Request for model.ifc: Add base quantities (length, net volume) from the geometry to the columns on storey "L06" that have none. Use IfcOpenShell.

First a look at what the model holds.

```python
import ifcopenshell
import ifcopenshell.util.element
import ifcopenshell.util.unit

model = ifcopenshell.open("model.ifc")
print(model.schema)
for unit_type in ("LENGTHUNIT", "AREAUNIT", "VOLUMEUNIT"):
    print(unit_type, ifcopenshell.util.unit.calculate_unit_scale(model, unit_type))
storey = next(s for s in model.by_type("IfcBuildingStorey") if s.Name == "L06")
columns = [e for e in ifcopenshell.util.element.get_decomposition(storey) if e.is_a("IfcColumn")]
for e in sorted(columns, key=lambda e: e.id()):
    print(e.id(), e.is_a(), e.Name, list(ifcopenshell.util.element.get_psets(e, qtos_only=True)), sep=" | ")
```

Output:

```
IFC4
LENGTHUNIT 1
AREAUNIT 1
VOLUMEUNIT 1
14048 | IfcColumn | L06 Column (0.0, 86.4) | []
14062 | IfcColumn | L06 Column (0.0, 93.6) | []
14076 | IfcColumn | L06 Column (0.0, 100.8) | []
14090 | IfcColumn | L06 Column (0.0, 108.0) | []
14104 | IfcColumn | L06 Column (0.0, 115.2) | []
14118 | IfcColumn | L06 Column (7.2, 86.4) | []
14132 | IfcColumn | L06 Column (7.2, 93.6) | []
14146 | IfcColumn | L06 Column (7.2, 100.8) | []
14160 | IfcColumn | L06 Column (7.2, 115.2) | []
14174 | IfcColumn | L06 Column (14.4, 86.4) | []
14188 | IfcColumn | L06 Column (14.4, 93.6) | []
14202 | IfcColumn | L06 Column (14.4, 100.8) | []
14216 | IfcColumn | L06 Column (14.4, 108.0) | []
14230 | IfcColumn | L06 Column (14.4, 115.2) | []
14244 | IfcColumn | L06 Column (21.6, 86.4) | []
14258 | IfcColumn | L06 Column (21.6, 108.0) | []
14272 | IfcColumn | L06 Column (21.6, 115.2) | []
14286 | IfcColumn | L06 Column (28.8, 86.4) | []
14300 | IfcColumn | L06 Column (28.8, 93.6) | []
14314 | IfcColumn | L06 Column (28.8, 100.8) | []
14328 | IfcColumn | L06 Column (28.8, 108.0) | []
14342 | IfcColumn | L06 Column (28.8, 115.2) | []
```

```python
import ifcopenshell
import ifcopenshell.api.pset
import ifcopenshell.geom
import ifcopenshell.util.element
import ifcopenshell.util.shape
import ifcopenshell.util.unit

model = ifcopenshell.open("model.ifc")
unit_scale = ifcopenshell.util.unit.calculate_unit_scale(model)
volume_scale = ifcopenshell.util.unit.calculate_unit_scale(model, "VOLUMEUNIT")
settings = ifcopenshell.geom.settings()

storey = next(s for s in model.by_type("IfcBuildingStorey") if s.Name == "L06")
columns = [e for e in ifcopenshell.util.element.get_decomposition(storey) if e.is_a("IfcColumn")]

for e in sorted(columns, key=lambda e: e.id()):
    if ifcopenshell.util.element.get_psets(e, qtos_only=True, should_inherit=False):
        continue
    # Geometry comes back in metres, in the element's own axes.
    shape = ifcopenshell.geom.create_shape(settings, e)
    values = {
        "Length": ifcopenshell.util.shape.get_z(shape.geometry) / unit_scale,
        "NetVolume": ifcopenshell.util.shape.get_volume(shape.geometry) / volume_scale,
    }
    qto = ifcopenshell.api.pset.add_qto(model, product=e, name="Qto_ColumnBaseQuantities")
    ifcopenshell.api.pset.edit_qto(model, qto=qto, properties=values)
    print(e.id(), {k: round(v, 3) for k, v in values.items()})

model.write("model_rev.ifc")
```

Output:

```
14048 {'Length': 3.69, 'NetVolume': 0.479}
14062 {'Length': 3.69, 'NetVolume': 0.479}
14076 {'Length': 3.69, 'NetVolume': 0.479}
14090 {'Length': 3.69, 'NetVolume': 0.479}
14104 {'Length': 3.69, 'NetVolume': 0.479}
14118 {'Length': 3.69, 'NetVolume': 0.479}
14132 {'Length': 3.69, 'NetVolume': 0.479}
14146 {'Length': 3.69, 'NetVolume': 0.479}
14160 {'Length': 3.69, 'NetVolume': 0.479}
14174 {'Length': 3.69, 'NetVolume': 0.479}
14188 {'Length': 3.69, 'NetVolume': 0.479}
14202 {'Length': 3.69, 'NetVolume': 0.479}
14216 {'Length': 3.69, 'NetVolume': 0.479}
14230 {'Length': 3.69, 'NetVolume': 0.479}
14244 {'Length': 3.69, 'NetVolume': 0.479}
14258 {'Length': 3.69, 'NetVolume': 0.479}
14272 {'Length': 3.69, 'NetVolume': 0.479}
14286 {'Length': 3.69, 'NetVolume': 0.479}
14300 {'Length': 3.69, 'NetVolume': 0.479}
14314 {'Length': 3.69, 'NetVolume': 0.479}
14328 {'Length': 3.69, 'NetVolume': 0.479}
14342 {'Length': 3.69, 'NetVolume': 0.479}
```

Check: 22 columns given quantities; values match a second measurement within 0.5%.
